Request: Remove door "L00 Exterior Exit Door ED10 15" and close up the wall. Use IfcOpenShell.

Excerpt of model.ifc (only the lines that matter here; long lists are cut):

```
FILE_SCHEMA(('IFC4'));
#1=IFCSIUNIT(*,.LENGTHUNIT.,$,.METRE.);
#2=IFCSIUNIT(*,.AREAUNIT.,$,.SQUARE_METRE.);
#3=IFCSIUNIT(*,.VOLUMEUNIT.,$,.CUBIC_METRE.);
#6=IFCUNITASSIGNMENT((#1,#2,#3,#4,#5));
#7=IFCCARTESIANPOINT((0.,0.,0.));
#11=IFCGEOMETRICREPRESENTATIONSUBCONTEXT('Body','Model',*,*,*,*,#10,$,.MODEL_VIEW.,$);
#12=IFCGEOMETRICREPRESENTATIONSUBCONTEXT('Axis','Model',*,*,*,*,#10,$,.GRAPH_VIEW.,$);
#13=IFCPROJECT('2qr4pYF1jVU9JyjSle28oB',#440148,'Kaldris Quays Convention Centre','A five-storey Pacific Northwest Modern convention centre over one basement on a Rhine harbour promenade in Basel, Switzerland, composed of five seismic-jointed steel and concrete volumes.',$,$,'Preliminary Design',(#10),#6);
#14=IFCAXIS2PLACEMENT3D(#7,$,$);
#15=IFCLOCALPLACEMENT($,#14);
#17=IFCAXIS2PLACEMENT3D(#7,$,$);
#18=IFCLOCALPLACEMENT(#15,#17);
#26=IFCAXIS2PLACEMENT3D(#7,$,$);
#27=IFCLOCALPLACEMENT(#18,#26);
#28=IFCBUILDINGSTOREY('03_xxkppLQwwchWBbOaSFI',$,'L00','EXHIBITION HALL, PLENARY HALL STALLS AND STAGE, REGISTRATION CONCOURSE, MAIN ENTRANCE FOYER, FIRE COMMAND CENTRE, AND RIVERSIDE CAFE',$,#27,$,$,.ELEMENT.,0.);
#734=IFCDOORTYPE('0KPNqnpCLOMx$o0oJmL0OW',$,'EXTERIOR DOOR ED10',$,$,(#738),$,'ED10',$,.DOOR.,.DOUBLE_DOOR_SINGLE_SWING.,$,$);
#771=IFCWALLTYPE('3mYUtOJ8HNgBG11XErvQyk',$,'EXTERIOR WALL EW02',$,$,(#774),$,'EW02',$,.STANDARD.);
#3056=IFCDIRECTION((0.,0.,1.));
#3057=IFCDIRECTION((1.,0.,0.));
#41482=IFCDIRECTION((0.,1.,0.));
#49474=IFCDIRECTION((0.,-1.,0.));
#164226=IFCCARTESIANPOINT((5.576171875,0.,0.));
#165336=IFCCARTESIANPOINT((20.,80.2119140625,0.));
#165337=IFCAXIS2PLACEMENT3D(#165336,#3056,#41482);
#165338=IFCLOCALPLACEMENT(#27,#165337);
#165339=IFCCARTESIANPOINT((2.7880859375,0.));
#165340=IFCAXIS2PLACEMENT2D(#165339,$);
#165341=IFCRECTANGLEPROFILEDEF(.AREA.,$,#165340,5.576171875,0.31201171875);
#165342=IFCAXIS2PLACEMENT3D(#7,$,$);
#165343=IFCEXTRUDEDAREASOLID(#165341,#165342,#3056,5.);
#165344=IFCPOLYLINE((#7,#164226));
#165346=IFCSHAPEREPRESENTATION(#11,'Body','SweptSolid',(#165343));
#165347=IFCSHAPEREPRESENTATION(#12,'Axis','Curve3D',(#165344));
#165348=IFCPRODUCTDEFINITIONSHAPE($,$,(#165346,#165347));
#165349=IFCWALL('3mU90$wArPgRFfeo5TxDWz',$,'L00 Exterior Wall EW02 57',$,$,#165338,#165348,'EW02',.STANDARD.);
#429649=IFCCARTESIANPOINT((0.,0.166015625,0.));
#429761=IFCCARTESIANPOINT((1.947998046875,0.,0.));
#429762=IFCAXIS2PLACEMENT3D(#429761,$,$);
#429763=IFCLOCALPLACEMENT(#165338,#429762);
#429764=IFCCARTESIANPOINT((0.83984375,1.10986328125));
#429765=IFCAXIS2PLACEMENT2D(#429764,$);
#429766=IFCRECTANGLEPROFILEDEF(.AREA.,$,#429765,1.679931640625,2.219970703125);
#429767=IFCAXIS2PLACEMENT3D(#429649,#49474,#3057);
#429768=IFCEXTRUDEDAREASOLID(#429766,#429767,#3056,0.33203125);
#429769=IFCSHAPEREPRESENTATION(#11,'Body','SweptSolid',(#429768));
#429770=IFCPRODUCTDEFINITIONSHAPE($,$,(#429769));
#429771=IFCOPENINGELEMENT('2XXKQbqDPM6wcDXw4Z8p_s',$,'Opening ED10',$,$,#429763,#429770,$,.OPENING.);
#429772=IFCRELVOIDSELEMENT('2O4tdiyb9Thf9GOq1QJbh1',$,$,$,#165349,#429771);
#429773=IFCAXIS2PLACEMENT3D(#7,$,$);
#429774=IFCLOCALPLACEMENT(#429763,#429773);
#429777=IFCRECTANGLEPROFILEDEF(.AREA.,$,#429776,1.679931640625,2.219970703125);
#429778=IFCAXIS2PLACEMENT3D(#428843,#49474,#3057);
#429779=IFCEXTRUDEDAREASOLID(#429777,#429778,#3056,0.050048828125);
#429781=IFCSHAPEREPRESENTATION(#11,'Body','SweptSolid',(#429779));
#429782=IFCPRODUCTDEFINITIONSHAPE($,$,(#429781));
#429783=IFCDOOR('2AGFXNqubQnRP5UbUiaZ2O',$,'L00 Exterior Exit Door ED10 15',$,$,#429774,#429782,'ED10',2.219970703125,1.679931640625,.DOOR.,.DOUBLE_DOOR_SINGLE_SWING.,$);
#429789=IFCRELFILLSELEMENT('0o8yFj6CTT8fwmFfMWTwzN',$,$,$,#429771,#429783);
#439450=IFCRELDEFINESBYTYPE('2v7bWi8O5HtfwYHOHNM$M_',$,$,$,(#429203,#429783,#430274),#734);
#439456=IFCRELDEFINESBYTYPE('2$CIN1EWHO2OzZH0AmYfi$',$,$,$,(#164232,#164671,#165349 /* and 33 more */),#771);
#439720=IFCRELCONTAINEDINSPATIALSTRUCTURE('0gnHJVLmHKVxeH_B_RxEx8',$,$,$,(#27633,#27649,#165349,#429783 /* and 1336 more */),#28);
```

```python
import ifcopenshell
import ifcopenshell.api.feature
import ifcopenshell.api.root
import ifcopenshell.geom
import ifcopenshell.util.shape

model = ifcopenshell.open("model.ifc")
settings = ifcopenshell.geom.settings()


def volume(element):
    """Net volume in cubic metres, openings subtracted."""
    shape = ifcopenshell.geom.create_shape(settings, element)
    return ifcopenshell.util.shape.get_volume(shape.geometry)


door = model.by_id(429783)
opening = door.FillsVoids[0].RelatingOpeningElement
wall = opening.VoidsElements[0].RelatingBuildingElement
before = volume(wall)

ifcopenshell.api.root.remove_product(model, product=door)
ifcopenshell.api.feature.remove_feature(model, feature=opening)

after = volume(wall)

print(f"wall volume {before:.3f} -> {after:.3f} m3")

model.write("model-out.ifc")
```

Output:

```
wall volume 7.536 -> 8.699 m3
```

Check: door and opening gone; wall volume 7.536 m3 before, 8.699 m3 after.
